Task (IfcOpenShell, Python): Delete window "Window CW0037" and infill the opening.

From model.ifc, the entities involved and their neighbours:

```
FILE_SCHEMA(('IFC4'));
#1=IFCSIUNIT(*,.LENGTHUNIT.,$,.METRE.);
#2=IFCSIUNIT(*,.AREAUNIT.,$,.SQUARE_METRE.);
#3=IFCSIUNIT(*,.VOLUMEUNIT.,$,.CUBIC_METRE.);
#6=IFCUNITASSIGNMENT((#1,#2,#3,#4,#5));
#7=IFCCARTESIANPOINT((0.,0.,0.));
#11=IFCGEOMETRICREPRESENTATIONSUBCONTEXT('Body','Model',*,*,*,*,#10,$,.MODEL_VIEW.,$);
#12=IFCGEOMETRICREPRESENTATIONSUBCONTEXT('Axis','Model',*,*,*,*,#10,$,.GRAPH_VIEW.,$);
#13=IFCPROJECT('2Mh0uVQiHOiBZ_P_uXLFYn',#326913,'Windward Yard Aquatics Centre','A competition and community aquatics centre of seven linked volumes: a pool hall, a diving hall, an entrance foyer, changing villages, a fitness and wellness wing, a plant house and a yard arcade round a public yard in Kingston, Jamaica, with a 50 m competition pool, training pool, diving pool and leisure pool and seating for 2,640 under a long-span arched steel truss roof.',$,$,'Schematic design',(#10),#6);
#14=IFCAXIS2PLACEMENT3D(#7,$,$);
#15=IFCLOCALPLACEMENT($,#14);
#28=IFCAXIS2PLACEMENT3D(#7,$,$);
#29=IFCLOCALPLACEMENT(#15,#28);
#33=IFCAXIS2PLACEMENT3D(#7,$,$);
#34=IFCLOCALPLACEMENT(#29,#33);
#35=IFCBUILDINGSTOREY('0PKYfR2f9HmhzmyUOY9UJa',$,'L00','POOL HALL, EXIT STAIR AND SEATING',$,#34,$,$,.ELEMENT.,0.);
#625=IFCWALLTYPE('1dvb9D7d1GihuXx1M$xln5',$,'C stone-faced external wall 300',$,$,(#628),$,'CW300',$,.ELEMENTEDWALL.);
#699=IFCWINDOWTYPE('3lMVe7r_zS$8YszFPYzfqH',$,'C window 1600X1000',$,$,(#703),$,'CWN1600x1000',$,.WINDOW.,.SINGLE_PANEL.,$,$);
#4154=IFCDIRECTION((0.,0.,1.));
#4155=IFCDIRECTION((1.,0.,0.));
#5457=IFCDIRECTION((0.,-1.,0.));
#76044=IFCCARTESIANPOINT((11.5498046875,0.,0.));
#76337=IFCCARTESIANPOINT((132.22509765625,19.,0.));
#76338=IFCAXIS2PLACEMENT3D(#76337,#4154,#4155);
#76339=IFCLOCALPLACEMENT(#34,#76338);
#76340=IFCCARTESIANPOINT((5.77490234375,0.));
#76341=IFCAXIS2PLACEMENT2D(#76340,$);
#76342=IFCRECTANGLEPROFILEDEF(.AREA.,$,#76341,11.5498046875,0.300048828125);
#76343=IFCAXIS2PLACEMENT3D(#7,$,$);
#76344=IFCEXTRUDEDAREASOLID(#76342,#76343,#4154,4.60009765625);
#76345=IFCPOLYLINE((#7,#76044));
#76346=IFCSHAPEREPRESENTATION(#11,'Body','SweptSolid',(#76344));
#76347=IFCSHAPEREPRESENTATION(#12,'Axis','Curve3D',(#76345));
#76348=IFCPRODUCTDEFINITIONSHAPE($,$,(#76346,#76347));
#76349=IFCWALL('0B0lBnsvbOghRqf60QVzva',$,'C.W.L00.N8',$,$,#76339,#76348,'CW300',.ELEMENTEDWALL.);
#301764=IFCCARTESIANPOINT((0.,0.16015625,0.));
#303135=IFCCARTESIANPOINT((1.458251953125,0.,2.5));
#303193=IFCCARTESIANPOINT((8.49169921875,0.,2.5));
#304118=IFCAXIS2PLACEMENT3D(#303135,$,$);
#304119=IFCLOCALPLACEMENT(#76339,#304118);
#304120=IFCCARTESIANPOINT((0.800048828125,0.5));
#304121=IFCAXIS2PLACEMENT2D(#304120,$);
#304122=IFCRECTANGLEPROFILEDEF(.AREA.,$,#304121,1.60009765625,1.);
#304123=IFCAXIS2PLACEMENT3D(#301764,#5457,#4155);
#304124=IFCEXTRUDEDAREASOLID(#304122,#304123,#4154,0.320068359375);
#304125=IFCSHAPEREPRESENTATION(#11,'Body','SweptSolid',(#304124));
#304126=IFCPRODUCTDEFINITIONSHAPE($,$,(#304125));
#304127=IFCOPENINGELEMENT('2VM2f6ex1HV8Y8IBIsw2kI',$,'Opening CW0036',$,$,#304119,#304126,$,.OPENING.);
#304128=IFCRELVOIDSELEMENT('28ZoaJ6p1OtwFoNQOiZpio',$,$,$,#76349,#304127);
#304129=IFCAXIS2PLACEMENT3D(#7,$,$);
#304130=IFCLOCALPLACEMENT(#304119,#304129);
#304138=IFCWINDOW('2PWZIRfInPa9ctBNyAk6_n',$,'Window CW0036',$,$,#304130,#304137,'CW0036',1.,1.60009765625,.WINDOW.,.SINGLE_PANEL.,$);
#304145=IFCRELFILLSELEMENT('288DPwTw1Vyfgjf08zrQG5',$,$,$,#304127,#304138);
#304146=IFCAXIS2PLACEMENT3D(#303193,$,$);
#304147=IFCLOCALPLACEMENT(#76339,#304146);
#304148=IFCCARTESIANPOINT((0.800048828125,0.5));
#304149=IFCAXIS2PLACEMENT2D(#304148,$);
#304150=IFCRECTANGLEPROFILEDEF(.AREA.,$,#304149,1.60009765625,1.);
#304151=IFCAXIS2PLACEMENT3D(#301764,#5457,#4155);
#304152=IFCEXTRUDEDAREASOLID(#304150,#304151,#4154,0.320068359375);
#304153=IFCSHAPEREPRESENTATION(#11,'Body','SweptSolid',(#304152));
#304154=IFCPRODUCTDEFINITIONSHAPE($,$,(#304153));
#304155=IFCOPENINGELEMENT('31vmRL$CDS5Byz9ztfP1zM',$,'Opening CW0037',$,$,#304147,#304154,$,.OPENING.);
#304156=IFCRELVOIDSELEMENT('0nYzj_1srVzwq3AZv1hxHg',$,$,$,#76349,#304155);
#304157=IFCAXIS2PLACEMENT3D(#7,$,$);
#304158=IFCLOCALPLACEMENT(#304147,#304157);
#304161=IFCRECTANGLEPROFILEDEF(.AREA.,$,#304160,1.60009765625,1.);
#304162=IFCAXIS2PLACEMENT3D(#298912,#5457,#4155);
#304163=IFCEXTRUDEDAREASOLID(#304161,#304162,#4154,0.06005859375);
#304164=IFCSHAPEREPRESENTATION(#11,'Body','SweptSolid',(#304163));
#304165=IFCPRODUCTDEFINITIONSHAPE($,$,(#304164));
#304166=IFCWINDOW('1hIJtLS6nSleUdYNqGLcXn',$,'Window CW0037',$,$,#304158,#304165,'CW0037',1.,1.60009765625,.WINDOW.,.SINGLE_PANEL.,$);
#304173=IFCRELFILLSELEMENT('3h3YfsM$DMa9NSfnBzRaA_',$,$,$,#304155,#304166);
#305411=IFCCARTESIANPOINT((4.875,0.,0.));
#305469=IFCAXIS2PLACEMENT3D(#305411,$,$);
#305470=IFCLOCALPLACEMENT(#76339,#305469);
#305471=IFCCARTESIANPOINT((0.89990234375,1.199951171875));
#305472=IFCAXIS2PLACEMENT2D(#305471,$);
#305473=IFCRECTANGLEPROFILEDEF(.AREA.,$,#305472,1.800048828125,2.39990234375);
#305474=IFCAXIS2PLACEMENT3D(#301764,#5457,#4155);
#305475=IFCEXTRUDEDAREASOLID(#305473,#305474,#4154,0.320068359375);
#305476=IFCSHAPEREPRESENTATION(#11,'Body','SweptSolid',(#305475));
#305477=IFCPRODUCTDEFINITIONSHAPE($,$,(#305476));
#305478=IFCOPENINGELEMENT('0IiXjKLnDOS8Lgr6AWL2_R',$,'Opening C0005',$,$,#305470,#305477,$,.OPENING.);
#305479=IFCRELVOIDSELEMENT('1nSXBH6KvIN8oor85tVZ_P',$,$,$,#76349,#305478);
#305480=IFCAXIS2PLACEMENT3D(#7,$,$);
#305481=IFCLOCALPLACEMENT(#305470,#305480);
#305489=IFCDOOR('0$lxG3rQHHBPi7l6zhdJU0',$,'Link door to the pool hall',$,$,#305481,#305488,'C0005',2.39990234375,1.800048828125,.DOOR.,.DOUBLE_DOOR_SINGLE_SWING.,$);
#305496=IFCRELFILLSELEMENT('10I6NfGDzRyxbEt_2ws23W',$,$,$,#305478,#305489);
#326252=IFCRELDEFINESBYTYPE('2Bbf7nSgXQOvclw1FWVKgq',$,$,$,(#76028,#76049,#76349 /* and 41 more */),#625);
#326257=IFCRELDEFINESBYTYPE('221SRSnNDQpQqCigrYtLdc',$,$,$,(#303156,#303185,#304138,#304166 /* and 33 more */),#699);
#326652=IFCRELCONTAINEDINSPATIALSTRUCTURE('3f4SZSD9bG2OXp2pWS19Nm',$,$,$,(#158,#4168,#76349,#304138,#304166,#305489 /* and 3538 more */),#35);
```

```python
import ifcopenshell
import ifcopenshell.api.feature
import ifcopenshell.api.root
import ifcopenshell.geom
import ifcopenshell.util.shape

model = ifcopenshell.open("model.ifc")
settings = ifcopenshell.geom.settings()


def volume(element):
    """Net volume in cubic metres, openings subtracted."""
    shape = ifcopenshell.geom.create_shape(settings, element)
    return ifcopenshell.util.shape.get_volume(shape.geometry)


window = model.by_guid("1hIJtLS6nSleUdYNqGLcXn")
opening = window.FillsVoids[0].RelatingOpeningElement
wall = opening.VoidsElements[0].RelatingBuildingElement
before = volume(wall)

ifcopenshell.api.root.remove_product(model, product=window)
ifcopenshell.api.feature.remove_feature(model, feature=opening)

after = volume(wall)

print(f"wall volume {before:.3f} -> {after:.3f} m3")

model.write("model_v2.ifc")
```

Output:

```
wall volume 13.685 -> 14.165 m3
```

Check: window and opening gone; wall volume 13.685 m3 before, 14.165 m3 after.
